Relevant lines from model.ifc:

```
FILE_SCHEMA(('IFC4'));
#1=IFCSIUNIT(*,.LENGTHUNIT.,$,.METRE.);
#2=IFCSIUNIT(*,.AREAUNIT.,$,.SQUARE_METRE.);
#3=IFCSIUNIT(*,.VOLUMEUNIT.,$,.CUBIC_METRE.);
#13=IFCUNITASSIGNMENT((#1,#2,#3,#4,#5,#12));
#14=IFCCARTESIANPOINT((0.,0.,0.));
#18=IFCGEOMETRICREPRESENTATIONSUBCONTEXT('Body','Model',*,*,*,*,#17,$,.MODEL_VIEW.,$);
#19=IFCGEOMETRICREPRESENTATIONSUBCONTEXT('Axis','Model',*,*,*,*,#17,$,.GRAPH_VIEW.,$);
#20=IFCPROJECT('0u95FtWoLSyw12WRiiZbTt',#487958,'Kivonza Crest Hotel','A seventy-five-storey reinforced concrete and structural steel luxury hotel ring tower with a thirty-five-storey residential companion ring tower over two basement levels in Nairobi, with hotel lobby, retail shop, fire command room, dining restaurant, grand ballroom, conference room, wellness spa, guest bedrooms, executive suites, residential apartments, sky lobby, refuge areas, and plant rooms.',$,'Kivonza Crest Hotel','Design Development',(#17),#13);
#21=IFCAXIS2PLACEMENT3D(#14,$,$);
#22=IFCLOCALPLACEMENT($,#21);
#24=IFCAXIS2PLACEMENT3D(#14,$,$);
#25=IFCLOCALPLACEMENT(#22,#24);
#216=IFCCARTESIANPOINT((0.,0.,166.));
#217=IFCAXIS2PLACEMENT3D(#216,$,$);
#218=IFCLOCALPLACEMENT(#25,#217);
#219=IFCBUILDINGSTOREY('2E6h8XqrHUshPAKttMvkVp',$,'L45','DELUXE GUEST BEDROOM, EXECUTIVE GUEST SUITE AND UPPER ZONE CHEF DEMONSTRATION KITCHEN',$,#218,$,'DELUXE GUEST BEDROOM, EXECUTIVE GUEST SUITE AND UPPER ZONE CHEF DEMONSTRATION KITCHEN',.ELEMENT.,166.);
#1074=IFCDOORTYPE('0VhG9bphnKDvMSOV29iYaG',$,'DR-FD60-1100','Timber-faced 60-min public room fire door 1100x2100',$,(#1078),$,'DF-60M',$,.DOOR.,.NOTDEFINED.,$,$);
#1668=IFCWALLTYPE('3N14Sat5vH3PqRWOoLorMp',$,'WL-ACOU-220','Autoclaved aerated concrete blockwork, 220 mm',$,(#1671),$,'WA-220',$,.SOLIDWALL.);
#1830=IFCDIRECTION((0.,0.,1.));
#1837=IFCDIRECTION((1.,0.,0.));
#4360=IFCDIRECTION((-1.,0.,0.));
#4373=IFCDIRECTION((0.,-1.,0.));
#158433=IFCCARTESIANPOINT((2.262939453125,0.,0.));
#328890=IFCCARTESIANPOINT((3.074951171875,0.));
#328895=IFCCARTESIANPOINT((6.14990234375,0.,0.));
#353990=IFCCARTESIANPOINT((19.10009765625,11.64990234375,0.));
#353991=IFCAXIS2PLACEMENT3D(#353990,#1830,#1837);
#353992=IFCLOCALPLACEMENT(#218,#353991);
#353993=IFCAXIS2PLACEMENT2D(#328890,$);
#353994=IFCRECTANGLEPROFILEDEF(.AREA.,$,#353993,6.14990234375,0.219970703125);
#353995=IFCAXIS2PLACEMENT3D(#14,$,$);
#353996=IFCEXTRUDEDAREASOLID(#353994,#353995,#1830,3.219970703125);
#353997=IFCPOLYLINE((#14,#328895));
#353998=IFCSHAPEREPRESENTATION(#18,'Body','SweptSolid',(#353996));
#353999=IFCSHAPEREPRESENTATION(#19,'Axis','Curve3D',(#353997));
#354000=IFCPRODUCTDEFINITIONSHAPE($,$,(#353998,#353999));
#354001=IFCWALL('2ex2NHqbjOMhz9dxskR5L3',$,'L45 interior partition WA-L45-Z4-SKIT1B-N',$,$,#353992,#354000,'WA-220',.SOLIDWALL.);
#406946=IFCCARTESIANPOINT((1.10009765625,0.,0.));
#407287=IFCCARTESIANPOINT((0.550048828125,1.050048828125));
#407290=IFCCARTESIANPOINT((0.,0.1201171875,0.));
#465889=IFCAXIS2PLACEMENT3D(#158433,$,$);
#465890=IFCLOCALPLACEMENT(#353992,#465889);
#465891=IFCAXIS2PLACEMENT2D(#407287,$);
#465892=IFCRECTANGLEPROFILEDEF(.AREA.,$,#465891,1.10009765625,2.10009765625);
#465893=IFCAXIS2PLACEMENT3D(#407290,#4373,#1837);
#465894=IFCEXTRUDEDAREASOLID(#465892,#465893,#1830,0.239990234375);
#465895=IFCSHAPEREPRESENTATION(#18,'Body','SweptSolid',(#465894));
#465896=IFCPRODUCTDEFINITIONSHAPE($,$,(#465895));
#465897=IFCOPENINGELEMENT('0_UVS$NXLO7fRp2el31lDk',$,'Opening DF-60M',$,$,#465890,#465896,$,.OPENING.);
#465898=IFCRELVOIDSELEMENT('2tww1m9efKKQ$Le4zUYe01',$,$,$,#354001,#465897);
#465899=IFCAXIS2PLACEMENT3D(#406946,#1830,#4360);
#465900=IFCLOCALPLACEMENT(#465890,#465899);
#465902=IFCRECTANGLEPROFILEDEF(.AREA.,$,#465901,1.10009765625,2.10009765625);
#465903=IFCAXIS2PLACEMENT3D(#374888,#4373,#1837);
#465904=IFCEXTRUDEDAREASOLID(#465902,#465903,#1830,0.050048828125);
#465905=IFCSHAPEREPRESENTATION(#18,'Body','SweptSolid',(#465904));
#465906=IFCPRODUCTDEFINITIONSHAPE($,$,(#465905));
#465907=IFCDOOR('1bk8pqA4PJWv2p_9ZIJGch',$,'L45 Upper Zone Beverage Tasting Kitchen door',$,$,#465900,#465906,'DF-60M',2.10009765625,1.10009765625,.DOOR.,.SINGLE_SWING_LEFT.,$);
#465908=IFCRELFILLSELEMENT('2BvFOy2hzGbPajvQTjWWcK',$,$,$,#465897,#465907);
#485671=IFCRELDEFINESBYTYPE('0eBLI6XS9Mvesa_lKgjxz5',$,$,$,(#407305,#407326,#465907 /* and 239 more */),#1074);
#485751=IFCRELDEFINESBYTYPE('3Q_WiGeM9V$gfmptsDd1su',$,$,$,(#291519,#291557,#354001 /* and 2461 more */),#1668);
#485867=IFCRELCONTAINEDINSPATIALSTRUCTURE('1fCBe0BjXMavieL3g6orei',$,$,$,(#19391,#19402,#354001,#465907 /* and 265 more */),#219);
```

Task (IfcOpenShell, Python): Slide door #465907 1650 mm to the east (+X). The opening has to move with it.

```python
import ifcopenshell
import ifcopenshell.api.geometry
import ifcopenshell.util.placement
import ifcopenshell.util.unit

model = ifcopenshell.open("model.ifc")
unit_scale = ifcopenshell.util.unit.calculate_unit_scale(model)

door = model.by_guid("1bk8pqA4PJWv2p_9ZIJGch")
opening = door.FillsVoids[0].RelatingOpeningElement
wall = opening.VoidsElements[0].RelatingBuildingElement

wall_matrix = ifcopenshell.util.placement.get_local_placement(wall.ObjectPlacement)
shift = wall_matrix[:3, 0] * 1.65 / unit_scale
before = ifcopenshell.util.placement.get_local_placement(door.ObjectPlacement)[:3, 3].copy()

# The door is placed relative to its opening, so it follows when the opening moves.
matrix = ifcopenshell.util.placement.get_local_placement(opening.ObjectPlacement)
matrix[:3, 3] += shift
ifcopenshell.api.geometry.edit_object_placement(
    model, product=opening, matrix=matrix, is_si=False, should_transform_children=True
)

after = ifcopenshell.util.placement.get_local_placement(door.ObjectPlacement)[:3, 3]
print("door moved by", (after - before).round(3) + 0.0)

model.write("model_v2.ifc")
```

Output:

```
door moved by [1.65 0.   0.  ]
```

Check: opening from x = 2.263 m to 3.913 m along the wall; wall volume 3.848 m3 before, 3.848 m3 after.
